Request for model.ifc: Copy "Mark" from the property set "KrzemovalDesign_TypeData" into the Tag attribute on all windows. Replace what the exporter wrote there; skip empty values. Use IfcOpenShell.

First a look at what the model holds.

```python
import ifcopenshell
import ifcopenshell.util.element

model = ifcopenshell.open("model.ifc")
print(model.schema)
windows = model.by_type("IfcWindow")
print(len(windows), "windows")
for e in windows[:8]:
    source = ifcopenshell.util.element.get_pset(e, "KrzemovalDesign_TypeData", "Mark")
    target = e.Tag
    print(e.id(), repr(source), repr(target), sep=" | ")
```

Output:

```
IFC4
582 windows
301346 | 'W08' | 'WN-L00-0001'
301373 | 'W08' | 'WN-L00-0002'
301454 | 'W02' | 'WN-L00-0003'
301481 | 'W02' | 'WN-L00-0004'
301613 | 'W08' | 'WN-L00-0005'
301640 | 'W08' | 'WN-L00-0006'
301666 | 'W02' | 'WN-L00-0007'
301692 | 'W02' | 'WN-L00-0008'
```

```python
import ifcopenshell
import ifcopenshell.util.element

model = ifcopenshell.open("model.ifc")

count = 0
for e in model.by_type("IfcWindow"):
    value = ifcopenshell.util.element.get_pset(e, "KrzemovalDesign_TypeData", "Mark")
    current = e.Tag
    if not value or not value.strip() or current == value:
        continue
    e.Tag = value
    count += 1

print(count, "windows updated")

model.write("model_v2.ifc")
```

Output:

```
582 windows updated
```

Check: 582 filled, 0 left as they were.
